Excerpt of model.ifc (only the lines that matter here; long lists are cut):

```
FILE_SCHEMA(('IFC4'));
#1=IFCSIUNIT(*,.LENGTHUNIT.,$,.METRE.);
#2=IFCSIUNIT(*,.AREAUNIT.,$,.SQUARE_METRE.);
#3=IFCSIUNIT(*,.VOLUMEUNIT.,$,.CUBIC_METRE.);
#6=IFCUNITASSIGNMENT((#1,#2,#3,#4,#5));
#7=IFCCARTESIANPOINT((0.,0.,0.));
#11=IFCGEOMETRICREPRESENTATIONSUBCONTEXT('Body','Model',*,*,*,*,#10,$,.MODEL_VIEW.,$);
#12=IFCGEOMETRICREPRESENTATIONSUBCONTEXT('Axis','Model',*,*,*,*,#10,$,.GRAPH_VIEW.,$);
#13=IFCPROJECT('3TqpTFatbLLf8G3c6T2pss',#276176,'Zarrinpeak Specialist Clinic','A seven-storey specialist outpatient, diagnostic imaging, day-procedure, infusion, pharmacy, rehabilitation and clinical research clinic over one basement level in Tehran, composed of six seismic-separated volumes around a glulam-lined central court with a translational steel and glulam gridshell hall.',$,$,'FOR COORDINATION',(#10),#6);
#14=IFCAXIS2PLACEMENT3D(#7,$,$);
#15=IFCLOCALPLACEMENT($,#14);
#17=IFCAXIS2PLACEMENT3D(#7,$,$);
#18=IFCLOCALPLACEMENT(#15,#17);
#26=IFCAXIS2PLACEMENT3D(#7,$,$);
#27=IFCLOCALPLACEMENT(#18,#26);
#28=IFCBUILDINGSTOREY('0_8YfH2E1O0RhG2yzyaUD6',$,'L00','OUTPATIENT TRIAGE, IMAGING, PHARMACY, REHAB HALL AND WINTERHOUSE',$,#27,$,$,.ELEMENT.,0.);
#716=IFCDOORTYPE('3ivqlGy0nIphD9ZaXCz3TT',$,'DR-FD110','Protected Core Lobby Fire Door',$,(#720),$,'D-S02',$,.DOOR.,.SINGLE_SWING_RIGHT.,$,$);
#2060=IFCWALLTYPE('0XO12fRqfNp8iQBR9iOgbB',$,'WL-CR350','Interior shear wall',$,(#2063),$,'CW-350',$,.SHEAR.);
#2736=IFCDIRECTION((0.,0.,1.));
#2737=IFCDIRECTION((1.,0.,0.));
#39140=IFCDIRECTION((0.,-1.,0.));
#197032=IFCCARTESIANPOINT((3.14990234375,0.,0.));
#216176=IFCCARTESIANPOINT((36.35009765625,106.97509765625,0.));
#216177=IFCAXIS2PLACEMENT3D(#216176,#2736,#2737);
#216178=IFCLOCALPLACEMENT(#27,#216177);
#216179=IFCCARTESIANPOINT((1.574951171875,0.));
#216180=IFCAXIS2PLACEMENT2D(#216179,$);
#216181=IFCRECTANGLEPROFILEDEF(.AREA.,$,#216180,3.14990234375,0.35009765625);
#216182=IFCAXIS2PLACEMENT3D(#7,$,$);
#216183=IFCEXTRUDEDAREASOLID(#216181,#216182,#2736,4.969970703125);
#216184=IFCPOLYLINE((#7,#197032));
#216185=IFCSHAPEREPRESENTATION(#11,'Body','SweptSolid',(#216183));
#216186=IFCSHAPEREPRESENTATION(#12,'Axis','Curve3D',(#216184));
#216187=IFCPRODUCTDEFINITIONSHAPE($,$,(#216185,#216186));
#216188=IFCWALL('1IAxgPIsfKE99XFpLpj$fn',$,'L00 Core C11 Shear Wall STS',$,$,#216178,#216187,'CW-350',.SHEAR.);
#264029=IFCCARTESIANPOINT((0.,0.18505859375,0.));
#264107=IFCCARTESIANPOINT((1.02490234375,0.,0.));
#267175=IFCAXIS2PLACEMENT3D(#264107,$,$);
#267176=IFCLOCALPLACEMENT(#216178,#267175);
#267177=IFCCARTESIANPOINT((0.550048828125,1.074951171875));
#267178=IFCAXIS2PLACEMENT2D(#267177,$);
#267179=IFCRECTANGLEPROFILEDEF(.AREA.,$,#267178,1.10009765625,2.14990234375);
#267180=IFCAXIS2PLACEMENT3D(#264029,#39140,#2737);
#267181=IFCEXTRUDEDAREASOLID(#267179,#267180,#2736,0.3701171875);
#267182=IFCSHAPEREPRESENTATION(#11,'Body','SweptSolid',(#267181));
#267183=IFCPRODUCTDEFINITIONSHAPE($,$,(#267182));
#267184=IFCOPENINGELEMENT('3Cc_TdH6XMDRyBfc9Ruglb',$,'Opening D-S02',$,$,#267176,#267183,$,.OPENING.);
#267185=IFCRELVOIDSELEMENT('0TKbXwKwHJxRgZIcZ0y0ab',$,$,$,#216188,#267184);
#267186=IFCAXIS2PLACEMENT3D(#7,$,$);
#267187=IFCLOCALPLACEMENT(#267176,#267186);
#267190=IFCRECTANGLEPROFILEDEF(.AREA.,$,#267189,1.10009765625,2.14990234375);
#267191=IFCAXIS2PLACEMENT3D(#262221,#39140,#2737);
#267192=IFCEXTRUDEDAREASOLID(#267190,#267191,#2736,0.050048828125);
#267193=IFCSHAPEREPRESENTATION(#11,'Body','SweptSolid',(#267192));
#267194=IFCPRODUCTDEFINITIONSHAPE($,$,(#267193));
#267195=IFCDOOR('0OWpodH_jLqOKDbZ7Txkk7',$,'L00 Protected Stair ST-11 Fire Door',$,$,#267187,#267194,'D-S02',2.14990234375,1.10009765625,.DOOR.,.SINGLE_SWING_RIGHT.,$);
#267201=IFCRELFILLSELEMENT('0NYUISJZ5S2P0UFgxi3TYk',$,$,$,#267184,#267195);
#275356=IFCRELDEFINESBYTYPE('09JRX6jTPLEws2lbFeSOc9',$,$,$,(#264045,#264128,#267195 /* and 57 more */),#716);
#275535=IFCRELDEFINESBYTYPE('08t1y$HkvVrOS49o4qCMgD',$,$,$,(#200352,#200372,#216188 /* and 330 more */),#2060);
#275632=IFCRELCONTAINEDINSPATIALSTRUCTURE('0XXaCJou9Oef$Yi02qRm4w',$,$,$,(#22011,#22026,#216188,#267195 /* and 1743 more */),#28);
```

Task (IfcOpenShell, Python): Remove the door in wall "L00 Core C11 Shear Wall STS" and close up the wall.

```python
import ifcopenshell
import ifcopenshell.api.feature
import ifcopenshell.api.root
import ifcopenshell.geom
import ifcopenshell.util.shape

model = ifcopenshell.open("model.ifc")
settings = ifcopenshell.geom.settings()


def volume(element):
    """Net volume in cubic metres, openings subtracted."""
    shape = ifcopenshell.geom.create_shape(settings, element)
    return ifcopenshell.util.shape.get_volume(shape.geometry)


door = model.by_guid("0OWpodH_jLqOKDbZ7Txkk7")
opening = door.FillsVoids[0].RelatingOpeningElement
wall = opening.VoidsElements[0].RelatingBuildingElement
before = volume(wall)

ifcopenshell.api.root.remove_product(model, product=door)
ifcopenshell.api.feature.remove_feature(model, feature=opening)

after = volume(wall)

print(f"wall volume {before:.3f} -> {after:.3f} m3")

model.write("model_updated.ifc")
```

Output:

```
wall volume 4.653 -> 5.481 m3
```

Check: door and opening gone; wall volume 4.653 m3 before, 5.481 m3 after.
